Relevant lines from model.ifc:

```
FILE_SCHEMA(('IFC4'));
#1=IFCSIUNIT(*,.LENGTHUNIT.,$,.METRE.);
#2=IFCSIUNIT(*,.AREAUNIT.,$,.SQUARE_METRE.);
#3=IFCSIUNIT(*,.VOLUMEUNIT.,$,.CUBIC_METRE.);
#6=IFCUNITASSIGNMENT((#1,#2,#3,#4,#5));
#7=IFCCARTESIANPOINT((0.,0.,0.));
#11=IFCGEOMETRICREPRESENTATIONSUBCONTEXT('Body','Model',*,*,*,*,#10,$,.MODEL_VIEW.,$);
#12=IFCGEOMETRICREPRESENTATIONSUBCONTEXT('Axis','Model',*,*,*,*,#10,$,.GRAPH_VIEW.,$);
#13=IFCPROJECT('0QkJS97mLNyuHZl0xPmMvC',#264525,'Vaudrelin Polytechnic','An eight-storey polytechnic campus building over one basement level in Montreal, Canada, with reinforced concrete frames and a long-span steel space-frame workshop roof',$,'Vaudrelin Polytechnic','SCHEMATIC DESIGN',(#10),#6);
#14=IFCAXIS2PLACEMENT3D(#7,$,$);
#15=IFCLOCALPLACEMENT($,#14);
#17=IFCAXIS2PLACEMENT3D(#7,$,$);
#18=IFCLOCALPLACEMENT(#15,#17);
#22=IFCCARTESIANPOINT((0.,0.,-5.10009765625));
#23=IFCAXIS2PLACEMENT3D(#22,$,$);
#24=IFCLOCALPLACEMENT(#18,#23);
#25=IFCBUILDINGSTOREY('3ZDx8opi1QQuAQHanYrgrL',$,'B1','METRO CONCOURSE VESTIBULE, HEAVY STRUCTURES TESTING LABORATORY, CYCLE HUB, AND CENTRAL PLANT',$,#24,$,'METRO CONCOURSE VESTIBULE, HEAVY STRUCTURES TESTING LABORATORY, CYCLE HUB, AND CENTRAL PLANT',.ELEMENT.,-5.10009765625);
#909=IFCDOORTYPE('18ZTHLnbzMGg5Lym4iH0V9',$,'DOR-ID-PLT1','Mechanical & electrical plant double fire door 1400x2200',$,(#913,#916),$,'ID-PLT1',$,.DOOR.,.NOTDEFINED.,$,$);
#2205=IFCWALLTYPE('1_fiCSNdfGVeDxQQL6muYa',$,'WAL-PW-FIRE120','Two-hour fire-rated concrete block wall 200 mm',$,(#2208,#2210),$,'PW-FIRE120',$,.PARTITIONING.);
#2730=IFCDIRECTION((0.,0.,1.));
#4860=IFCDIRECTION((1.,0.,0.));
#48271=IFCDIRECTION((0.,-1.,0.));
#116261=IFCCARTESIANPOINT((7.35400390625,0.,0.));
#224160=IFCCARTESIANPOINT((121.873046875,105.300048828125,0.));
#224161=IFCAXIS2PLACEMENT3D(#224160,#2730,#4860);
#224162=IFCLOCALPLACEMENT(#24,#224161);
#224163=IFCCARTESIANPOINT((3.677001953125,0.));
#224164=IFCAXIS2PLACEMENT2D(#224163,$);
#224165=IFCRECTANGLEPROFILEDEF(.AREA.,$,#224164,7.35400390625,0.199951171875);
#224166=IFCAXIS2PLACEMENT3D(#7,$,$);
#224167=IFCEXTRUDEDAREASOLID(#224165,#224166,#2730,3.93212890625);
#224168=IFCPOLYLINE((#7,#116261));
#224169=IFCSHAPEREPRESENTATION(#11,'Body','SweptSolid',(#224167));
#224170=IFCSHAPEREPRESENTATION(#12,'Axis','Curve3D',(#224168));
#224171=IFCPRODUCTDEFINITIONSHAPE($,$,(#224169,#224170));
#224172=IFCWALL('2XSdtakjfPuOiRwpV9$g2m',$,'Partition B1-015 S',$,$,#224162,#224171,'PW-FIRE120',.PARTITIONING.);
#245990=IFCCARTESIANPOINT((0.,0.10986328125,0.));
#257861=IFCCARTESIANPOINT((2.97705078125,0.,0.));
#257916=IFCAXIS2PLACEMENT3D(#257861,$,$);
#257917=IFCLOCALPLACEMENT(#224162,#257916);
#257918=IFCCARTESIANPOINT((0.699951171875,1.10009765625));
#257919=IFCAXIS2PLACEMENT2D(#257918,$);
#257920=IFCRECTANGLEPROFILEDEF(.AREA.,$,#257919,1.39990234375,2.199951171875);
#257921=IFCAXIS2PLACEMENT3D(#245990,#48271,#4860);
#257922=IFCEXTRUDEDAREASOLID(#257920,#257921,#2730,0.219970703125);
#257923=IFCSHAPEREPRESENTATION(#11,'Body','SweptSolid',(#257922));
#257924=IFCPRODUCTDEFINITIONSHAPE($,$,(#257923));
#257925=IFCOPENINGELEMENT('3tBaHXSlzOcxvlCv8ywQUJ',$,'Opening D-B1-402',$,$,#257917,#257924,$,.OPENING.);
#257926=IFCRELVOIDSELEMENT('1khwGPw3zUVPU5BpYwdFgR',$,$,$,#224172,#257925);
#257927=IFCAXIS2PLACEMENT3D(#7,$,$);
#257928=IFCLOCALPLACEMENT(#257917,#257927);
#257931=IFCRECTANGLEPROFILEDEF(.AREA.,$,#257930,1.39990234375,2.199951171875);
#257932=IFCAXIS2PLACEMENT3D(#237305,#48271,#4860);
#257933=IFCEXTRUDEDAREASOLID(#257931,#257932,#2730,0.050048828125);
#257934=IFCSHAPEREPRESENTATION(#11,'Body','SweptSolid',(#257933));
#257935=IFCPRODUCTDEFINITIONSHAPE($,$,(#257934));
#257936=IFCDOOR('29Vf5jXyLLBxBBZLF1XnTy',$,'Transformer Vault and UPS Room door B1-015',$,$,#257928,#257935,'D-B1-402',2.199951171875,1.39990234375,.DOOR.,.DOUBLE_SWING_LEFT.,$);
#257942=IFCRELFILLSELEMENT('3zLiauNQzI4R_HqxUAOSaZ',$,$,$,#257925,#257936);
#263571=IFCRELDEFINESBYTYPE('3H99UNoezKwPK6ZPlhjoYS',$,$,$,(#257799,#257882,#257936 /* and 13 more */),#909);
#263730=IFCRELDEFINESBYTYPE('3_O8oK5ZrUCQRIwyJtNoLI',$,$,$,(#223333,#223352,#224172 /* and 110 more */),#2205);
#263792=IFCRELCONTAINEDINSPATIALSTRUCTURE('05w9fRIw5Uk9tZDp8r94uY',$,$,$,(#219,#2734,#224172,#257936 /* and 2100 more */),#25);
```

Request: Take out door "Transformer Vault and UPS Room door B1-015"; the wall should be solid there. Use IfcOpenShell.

```python
import ifcopenshell
import ifcopenshell.api.feature
import ifcopenshell.api.root
import ifcopenshell.geom
import ifcopenshell.util.shape

model = ifcopenshell.open("model.ifc")
settings = ifcopenshell.geom.settings()


def volume(element):
    """Net volume in cubic metres, openings subtracted."""
    shape = ifcopenshell.geom.create_shape(settings, element)
    return ifcopenshell.util.shape.get_volume(shape.geometry)


door = model.by_guid("29Vf5jXyLLBxBBZLF1XnTy")
opening = door.FillsVoids[0].RelatingOpeningElement
wall = opening.VoidsElements[0].RelatingBuildingElement
before = volume(wall)

ifcopenshell.api.root.remove_product(model, product=door)
ifcopenshell.api.feature.remove_feature(model, feature=opening)

after = volume(wall)

print(f"wall volume {before:.3f} -> {after:.3f} m3")

model.write("model-out.ifc")
```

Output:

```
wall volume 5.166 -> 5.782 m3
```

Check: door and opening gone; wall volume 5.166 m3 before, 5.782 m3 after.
